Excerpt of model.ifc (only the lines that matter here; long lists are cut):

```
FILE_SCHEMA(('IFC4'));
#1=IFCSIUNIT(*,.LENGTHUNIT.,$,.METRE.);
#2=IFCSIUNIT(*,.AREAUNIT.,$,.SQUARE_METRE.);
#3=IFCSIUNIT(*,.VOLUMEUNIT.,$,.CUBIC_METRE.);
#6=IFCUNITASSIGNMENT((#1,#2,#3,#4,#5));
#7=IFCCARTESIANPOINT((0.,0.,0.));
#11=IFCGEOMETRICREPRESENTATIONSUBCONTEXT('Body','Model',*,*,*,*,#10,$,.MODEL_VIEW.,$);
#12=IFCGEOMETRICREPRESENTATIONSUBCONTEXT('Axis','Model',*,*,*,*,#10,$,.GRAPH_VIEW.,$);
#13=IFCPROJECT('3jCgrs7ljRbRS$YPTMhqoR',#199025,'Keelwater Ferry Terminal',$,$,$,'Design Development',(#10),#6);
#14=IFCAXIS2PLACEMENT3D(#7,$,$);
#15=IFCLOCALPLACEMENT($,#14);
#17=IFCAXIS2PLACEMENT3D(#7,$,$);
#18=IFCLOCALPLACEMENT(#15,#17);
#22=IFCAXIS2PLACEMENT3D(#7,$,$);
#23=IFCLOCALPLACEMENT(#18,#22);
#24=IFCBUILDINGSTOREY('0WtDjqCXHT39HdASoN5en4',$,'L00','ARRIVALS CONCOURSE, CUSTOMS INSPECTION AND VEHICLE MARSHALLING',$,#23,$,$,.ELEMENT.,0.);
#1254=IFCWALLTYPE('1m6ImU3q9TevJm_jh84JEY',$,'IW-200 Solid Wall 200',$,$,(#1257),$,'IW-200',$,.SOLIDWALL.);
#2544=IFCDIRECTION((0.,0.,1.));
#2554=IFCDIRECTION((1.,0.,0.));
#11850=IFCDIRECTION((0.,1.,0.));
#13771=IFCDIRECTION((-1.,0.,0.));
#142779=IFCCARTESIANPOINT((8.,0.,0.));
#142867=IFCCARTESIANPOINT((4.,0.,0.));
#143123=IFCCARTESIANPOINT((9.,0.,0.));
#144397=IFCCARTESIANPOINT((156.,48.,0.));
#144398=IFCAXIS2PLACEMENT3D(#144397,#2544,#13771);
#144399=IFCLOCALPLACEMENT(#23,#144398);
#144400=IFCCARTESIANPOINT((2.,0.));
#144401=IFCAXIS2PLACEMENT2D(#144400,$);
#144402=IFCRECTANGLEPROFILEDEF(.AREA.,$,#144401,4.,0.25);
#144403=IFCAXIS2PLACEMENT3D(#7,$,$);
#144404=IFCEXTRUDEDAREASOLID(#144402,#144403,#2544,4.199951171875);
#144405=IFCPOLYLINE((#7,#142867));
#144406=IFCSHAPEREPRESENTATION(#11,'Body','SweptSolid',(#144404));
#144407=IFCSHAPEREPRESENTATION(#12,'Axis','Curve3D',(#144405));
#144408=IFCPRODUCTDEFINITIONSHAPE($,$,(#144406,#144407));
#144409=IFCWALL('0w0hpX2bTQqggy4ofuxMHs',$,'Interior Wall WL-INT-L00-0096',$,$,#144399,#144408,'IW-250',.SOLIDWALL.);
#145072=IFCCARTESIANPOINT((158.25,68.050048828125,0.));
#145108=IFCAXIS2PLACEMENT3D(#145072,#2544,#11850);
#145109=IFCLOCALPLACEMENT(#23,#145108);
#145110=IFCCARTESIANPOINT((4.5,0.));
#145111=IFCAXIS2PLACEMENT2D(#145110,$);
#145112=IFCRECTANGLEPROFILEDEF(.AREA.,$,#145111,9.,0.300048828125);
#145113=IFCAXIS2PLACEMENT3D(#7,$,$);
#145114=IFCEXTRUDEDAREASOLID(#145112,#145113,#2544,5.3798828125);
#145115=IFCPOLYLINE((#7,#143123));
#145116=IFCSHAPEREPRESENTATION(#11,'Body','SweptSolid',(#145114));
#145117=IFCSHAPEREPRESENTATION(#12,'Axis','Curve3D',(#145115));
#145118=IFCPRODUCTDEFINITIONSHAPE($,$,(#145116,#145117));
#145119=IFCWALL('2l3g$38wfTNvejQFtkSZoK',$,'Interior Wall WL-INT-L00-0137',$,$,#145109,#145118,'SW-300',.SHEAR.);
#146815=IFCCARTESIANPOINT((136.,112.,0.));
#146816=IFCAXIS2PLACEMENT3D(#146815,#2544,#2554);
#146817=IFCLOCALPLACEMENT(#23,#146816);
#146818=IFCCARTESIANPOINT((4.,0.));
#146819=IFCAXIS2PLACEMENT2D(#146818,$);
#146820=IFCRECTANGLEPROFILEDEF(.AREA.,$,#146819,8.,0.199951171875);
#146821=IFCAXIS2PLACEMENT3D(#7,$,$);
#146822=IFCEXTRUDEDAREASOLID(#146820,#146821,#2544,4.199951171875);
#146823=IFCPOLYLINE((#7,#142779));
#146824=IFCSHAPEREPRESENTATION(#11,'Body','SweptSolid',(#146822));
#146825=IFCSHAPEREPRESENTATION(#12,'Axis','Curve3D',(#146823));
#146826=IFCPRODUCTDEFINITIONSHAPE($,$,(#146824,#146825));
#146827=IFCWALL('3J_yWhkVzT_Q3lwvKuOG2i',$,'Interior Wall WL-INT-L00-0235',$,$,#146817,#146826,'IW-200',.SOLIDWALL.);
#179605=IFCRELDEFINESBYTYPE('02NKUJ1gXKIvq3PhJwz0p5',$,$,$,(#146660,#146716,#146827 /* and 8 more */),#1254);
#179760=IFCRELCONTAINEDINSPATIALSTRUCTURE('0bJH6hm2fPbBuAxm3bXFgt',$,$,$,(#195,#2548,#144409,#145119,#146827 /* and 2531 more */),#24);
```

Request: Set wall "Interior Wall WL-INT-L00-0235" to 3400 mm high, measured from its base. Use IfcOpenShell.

```python
import ifcopenshell
import ifcopenshell.geom
import ifcopenshell.util.representation
import ifcopenshell.util.shape

model = ifcopenshell.open("model.ifc")
settings = ifcopenshell.geom.settings()


def volume(element):
    """Net volume in cubic metres, openings subtracted."""
    shape = ifcopenshell.geom.create_shape(settings, element)
    return ifcopenshell.util.shape.get_volume(shape.geometry)


wall = model.by_guid("3J_yWhkVzT_Q3lwvKuOG2i")
before = volume(wall)

body = ifcopenshell.util.representation.get_representation(wall, "Model", "Body")
solid = body.Items[0]
old_height = solid.Depth
solid.Depth = 3.4
after = volume(wall)

print(f"height {old_height:g} -> {solid.Depth:g}, volume {before:.3f} -> {after:.3f} m3")

model.write("model_edited.ifc")
```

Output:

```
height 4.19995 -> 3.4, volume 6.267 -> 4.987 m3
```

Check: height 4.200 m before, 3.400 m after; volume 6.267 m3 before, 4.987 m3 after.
